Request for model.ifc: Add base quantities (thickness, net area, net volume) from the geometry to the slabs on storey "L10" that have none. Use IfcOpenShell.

First a look at what the model holds.

```python
import ifcopenshell
import ifcopenshell.util.element
import ifcopenshell.util.unit

model = ifcopenshell.open("model.ifc")
print(model.schema)
for unit_type in ("LENGTHUNIT", "AREAUNIT", "VOLUMEUNIT"):
    print(unit_type, ifcopenshell.util.unit.calculate_unit_scale(model, unit_type))
storey = next(s for s in model.by_type("IfcBuildingStorey") if s.Name == "L10")
slabs = [e for e in ifcopenshell.util.element.get_decomposition(storey) if e.is_a("IfcSlab")]
for e in sorted(slabs, key=lambda e: e.id()):
    print(e.id(), e.is_a(), e.Name, list(ifcopenshell.util.element.get_psets(e, qtos_only=True)), sep=" | ")
```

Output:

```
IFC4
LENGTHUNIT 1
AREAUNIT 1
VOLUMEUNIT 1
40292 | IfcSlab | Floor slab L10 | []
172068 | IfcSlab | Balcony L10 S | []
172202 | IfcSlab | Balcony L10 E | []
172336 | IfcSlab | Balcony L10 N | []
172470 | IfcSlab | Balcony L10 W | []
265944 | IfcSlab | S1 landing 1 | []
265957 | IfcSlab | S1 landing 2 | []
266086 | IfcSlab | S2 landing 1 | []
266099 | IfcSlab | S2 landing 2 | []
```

```python
import ifcopenshell
import ifcopenshell.api.pset
import ifcopenshell.geom
import ifcopenshell.util.element
import ifcopenshell.util.shape
import ifcopenshell.util.unit

model = ifcopenshell.open("model.ifc")
unit_scale = ifcopenshell.util.unit.calculate_unit_scale(model)
area_scale = ifcopenshell.util.unit.calculate_unit_scale(model, "AREAUNIT")
volume_scale = ifcopenshell.util.unit.calculate_unit_scale(model, "VOLUMEUNIT")
settings = ifcopenshell.geom.settings()

storey = next(s for s in model.by_type("IfcBuildingStorey") if s.Name == "L10")
slabs = [e for e in ifcopenshell.util.element.get_decomposition(storey) if e.is_a("IfcSlab")]

for e in sorted(slabs, key=lambda e: e.id()):
    if ifcopenshell.util.element.get_psets(e, qtos_only=True, should_inherit=False):
        continue
    # Geometry comes back in metres, in the element's own axes.
    shape = ifcopenshell.geom.create_shape(settings, e)
    values = {
        "Width": ifcopenshell.util.shape.get_z(shape.geometry) / unit_scale,
        "NetArea": ifcopenshell.util.shape.get_footprint_area(shape.geometry) / area_scale,
        "NetVolume": ifcopenshell.util.shape.get_volume(shape.geometry) / volume_scale,
    }
    qto = ifcopenshell.api.pset.add_qto(model, product=e, name="Qto_SlabBaseQuantities")
    ifcopenshell.api.pset.edit_qto(model, qto=qto, properties=values)
    print(e.id(), {k: round(v, 3) for k, v in values.items()})

model.write("model_edited.ifc")
```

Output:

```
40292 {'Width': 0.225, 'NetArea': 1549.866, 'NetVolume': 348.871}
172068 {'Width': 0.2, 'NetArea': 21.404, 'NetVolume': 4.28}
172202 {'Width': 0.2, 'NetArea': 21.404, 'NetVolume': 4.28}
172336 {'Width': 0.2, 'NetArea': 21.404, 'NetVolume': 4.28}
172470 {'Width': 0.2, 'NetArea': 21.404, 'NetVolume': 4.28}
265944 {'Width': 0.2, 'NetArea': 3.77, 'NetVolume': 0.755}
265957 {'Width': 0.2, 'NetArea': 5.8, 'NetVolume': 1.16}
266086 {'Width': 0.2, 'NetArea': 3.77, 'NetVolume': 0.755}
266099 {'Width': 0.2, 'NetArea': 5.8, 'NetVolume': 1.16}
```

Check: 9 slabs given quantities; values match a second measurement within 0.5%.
